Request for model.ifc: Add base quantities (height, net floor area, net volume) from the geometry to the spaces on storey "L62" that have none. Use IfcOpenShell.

First a look at what the model holds.

```python
import ifcopenshell
import ifcopenshell.util.element
import ifcopenshell.util.unit

model = ifcopenshell.open("model.ifc")
print(model.schema)
for unit_type in ("LENGTHUNIT", "AREAUNIT", "VOLUMEUNIT"):
    print(unit_type, ifcopenshell.util.unit.calculate_unit_scale(model, unit_type))
storey = next(s for s in model.by_type("IfcBuildingStorey") if s.Name == "L62")
spaces = [e for e in ifcopenshell.util.element.get_decomposition(storey) if e.is_a("IfcSpace")]
for e in sorted(spaces, key=lambda e: e.id()):
    print(e.id(), e.is_a(), e.Name, list(ifcopenshell.util.element.get_psets(e, qtos_only=True)), sep=" | ")
```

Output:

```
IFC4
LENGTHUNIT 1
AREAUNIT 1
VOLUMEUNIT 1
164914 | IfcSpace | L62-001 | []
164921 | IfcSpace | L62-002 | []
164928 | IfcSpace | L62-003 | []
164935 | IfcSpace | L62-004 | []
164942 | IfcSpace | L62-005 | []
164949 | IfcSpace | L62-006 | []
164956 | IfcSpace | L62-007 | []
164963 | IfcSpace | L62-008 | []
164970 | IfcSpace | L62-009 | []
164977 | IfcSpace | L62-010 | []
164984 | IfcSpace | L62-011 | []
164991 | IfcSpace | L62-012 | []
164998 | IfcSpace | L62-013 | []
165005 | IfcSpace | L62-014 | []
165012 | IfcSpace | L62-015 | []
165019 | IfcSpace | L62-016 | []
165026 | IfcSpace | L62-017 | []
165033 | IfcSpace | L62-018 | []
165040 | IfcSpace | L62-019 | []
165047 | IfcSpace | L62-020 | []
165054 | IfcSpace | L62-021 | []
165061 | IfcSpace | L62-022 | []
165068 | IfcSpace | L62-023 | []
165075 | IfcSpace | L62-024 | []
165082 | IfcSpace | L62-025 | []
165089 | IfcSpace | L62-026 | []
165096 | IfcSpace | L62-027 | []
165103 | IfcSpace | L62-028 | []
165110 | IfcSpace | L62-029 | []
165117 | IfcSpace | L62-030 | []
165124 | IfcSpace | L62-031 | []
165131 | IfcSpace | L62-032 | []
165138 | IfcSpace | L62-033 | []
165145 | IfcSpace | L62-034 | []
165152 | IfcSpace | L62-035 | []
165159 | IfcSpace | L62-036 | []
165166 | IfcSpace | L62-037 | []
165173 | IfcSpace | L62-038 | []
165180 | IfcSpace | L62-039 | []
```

```python
import ifcopenshell
import ifcopenshell.api.pset
import ifcopenshell.geom
import ifcopenshell.util.element
import ifcopenshell.util.shape
import ifcopenshell.util.unit

model = ifcopenshell.open("model.ifc")
unit_scale = ifcopenshell.util.unit.calculate_unit_scale(model)
area_scale = ifcopenshell.util.unit.calculate_unit_scale(model, "AREAUNIT")
volume_scale = ifcopenshell.util.unit.calculate_unit_scale(model, "VOLUMEUNIT")
settings = ifcopenshell.geom.settings()

storey = next(s for s in model.by_type("IfcBuildingStorey") if s.Name == "L62")
spaces = [e for e in ifcopenshell.util.element.get_decomposition(storey) if e.is_a("IfcSpace")]

for e in sorted(spaces, key=lambda e: e.id()):
    if ifcopenshell.util.element.get_psets(e, qtos_only=True, should_inherit=False):
        continue
    # Geometry comes back in metres, in the element's own axes.
    shape = ifcopenshell.geom.create_shape(settings, e)
    values = {
        "Height": ifcopenshell.util.shape.get_z(shape.geometry) / unit_scale,
        "NetFloorArea": ifcopenshell.util.shape.get_footprint_area(shape.geometry) / area_scale,
        "NetVolume": ifcopenshell.util.shape.get_volume(shape.geometry) / volume_scale,
    }
    qto = ifcopenshell.api.pset.add_qto(model, product=e, name="Qto_SpaceBaseQuantities")
    ifcopenshell.api.pset.edit_qto(model, qto=qto, properties=values)
    print(e.id(), {k: round(v, 3) for k, v in values.items()})

model.write("model_updated.ifc")
```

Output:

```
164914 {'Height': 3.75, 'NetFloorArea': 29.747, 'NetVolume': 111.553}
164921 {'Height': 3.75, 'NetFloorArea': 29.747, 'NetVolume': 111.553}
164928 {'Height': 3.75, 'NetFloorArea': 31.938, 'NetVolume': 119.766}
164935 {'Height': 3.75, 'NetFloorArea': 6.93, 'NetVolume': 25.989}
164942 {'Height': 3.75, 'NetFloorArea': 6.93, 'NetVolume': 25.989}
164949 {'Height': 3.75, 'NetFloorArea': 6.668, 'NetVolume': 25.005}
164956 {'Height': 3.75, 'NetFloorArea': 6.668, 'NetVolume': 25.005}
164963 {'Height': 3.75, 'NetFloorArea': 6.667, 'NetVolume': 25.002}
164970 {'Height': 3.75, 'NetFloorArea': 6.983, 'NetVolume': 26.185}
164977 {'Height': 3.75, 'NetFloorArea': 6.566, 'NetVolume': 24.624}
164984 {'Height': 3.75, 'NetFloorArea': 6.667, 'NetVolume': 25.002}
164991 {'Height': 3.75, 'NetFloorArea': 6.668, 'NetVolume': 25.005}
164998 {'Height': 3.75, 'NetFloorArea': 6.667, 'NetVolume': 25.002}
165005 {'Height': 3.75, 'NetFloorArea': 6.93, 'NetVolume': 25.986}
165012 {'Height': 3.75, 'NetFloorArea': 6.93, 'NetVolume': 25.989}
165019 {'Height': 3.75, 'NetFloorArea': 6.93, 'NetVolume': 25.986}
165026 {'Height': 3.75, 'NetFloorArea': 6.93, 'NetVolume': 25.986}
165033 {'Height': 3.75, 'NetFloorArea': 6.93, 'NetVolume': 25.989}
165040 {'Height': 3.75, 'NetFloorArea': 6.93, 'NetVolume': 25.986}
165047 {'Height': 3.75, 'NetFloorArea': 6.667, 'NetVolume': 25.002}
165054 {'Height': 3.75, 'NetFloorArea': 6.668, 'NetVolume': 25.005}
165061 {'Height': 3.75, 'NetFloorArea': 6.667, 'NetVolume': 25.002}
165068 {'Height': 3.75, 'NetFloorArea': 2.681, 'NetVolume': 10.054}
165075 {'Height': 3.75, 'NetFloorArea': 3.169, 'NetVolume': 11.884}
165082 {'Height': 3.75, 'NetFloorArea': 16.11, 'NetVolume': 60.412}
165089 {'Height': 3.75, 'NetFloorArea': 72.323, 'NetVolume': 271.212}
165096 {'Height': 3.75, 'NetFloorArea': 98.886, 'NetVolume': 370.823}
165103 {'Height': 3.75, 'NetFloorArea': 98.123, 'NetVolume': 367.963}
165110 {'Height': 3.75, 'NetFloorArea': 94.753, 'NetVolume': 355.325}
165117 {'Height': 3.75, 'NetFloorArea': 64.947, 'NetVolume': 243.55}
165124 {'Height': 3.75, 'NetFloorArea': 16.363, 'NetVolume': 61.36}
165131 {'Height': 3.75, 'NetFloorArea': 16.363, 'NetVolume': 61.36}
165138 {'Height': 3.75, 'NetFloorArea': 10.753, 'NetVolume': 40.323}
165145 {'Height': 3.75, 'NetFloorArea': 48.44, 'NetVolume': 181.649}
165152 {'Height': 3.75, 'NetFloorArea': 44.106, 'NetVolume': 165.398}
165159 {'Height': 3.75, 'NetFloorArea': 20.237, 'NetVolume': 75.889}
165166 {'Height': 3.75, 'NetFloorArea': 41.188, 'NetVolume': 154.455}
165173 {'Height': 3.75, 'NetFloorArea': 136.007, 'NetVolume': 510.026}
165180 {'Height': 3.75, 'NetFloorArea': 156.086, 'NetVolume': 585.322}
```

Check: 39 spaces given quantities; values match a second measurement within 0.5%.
